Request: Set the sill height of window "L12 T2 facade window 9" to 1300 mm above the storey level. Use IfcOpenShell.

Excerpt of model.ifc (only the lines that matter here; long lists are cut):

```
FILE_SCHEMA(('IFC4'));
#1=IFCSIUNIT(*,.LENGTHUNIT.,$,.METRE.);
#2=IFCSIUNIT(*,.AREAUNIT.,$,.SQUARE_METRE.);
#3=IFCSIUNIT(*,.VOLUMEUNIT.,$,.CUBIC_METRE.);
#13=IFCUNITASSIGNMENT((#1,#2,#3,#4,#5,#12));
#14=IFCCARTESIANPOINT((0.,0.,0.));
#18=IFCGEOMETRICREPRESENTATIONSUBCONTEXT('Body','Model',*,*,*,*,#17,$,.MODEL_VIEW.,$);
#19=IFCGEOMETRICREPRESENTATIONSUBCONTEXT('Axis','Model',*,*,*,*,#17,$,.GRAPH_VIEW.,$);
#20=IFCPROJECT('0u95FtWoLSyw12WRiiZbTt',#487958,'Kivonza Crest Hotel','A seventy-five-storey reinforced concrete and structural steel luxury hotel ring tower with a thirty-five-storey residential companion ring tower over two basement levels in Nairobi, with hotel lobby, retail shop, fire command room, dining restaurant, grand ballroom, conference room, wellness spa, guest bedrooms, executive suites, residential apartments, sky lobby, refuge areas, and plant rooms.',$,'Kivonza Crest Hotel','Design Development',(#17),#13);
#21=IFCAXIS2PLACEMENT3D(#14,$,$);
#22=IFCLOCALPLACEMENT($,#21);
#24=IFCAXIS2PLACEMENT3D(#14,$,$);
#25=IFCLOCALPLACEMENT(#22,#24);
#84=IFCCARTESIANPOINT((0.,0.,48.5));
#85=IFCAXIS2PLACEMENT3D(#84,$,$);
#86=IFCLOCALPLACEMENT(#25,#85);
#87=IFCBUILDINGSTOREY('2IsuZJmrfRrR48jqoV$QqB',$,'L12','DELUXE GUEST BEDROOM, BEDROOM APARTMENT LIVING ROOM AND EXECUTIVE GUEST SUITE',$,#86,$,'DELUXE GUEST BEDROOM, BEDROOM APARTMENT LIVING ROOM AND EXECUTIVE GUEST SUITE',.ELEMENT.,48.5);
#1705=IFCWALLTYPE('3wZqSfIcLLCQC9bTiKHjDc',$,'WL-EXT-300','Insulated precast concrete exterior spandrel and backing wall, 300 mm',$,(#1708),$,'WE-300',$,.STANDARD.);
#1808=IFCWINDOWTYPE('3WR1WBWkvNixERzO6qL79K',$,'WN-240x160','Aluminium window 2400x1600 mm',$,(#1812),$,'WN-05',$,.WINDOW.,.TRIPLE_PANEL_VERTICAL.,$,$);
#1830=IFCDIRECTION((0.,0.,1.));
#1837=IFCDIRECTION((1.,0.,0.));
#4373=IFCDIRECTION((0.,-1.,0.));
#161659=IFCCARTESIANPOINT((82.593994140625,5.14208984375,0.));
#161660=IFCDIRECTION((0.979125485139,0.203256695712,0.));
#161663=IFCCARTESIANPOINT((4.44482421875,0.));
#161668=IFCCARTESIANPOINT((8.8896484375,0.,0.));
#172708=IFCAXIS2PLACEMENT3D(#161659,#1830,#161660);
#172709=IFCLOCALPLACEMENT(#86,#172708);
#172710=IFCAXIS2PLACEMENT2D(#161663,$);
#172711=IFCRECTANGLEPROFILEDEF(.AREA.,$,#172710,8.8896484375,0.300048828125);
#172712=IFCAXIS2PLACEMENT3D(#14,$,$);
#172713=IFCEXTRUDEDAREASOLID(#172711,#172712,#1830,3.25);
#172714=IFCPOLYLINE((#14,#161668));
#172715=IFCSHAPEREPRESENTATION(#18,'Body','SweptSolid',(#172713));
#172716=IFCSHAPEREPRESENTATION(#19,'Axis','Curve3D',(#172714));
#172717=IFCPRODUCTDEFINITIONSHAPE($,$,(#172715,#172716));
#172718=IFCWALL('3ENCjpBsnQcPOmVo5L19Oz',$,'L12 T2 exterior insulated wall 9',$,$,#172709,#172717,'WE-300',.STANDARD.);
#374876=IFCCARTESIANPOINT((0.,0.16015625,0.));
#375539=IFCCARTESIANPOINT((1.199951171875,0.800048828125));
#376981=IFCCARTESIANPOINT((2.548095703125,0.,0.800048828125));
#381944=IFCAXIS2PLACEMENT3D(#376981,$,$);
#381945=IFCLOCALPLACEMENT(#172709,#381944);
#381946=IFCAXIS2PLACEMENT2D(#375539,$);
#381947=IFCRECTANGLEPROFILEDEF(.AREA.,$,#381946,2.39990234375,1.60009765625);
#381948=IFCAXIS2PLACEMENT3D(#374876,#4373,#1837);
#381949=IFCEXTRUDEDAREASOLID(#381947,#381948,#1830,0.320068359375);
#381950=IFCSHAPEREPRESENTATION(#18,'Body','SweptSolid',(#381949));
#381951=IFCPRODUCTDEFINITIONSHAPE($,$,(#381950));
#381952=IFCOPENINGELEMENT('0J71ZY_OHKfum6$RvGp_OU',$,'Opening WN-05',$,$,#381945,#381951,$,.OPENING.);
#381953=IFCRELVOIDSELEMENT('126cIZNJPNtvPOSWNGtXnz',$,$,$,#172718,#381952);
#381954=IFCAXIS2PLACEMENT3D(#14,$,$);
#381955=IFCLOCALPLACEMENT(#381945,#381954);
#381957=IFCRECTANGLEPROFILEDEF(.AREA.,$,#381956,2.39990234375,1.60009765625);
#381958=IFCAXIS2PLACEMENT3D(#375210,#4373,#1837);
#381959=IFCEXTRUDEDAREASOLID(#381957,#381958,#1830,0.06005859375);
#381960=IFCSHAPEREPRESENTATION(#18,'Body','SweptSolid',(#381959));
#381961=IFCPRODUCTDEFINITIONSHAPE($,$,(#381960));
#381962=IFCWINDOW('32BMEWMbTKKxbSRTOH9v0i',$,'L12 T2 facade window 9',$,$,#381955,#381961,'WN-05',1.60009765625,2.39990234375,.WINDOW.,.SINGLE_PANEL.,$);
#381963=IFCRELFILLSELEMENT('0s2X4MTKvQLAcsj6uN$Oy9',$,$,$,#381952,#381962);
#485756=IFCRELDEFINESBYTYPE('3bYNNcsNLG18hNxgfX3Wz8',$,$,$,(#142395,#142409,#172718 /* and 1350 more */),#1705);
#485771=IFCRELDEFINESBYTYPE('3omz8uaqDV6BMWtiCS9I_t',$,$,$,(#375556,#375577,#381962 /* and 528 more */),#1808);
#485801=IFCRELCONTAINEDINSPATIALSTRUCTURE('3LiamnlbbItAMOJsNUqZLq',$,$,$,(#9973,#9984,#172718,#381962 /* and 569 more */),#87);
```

```python
import numpy as np
import ifcopenshell
import ifcopenshell.api.geometry
import ifcopenshell.geom
import ifcopenshell.util.element
import ifcopenshell.util.placement
import ifcopenshell.util.shape
import ifcopenshell.util.unit

model = ifcopenshell.open("model.ifc")
unit_scale = ifcopenshell.util.unit.calculate_unit_scale(model)

window = model.by_id(381962)
opening = window.FillsVoids[0].RelatingOpeningElement
storey = ifcopenshell.util.element.get_container(window, ifc_class="IfcBuildingStorey")
level = ifcopenshell.util.placement.get_local_placement(storey.ObjectPlacement)[2, 3]

# The opening's origin need not be at the sill, so measure its lowest point.
shape = ifcopenshell.geom.create_shape(ifcopenshell.geom.settings(), opening)
bottom = ifcopenshell.util.shape.get_shape_bottom_elevation(shape, shape.geometry) / unit_scale
dz = level + 1.3 / unit_scale - bottom

shift = np.array([0.0, 0.0, dz])
# The window is placed relative to its opening, so it follows when the opening moves.
matrix = ifcopenshell.util.placement.get_local_placement(opening.ObjectPlacement)
matrix[:3, 3] += shift
ifcopenshell.api.geometry.edit_object_placement(
    model, product=opening, matrix=matrix, is_si=False, should_transform_children=True
)

print(f"moved by {dz * unit_scale:+.3f} m")

model.write("model_updated.ifc")
```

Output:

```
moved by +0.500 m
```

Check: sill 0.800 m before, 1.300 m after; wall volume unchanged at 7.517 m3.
